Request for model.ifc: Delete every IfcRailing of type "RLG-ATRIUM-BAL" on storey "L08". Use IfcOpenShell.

First a look at what the model holds.

```python
import ifcopenshell
import ifcopenshell.util.element

model = ifcopenshell.open("model.ifc")
print(model.schema)
storey = next(s for s in model.by_type("IfcBuildingStorey") if s.Name == "L08")
railings = [e for e in ifcopenshell.util.element.get_decomposition(storey) if e.is_a("IfcRailing")]
seen = {}
for e in railings:
    element_type = ifcopenshell.util.element.get_type(e)
    name = element_type.Name if element_type not in (None, e) else None
    seen[name] = seen.get(name, 0) + 1
for name, count in sorted(seen.items(), key=str):
    print(count, "x", name)
```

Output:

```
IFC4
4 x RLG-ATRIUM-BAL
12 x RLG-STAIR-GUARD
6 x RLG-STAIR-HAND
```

```python
import ifcopenshell
import ifcopenshell.api.root
import ifcopenshell.util.element

model = ifcopenshell.open("model.ifc")

storey = next(s for s in model.by_type("IfcBuildingStorey") if s.Name == "L08")
railings = [e for e in ifcopenshell.util.element.get_decomposition(storey) if e.is_a("IfcRailing")]
targets = [e for e in railings if (t := ifcopenshell.util.element.get_type(e)) not in (None, e) and t.Name == "RLG-ATRIUM-BAL"]

for e in targets:
    ifcopenshell.api.root.remove_product(model, product=e)
print(len(targets), "removed")

model.write("model_updated.ifc")
```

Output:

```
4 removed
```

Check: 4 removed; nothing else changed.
